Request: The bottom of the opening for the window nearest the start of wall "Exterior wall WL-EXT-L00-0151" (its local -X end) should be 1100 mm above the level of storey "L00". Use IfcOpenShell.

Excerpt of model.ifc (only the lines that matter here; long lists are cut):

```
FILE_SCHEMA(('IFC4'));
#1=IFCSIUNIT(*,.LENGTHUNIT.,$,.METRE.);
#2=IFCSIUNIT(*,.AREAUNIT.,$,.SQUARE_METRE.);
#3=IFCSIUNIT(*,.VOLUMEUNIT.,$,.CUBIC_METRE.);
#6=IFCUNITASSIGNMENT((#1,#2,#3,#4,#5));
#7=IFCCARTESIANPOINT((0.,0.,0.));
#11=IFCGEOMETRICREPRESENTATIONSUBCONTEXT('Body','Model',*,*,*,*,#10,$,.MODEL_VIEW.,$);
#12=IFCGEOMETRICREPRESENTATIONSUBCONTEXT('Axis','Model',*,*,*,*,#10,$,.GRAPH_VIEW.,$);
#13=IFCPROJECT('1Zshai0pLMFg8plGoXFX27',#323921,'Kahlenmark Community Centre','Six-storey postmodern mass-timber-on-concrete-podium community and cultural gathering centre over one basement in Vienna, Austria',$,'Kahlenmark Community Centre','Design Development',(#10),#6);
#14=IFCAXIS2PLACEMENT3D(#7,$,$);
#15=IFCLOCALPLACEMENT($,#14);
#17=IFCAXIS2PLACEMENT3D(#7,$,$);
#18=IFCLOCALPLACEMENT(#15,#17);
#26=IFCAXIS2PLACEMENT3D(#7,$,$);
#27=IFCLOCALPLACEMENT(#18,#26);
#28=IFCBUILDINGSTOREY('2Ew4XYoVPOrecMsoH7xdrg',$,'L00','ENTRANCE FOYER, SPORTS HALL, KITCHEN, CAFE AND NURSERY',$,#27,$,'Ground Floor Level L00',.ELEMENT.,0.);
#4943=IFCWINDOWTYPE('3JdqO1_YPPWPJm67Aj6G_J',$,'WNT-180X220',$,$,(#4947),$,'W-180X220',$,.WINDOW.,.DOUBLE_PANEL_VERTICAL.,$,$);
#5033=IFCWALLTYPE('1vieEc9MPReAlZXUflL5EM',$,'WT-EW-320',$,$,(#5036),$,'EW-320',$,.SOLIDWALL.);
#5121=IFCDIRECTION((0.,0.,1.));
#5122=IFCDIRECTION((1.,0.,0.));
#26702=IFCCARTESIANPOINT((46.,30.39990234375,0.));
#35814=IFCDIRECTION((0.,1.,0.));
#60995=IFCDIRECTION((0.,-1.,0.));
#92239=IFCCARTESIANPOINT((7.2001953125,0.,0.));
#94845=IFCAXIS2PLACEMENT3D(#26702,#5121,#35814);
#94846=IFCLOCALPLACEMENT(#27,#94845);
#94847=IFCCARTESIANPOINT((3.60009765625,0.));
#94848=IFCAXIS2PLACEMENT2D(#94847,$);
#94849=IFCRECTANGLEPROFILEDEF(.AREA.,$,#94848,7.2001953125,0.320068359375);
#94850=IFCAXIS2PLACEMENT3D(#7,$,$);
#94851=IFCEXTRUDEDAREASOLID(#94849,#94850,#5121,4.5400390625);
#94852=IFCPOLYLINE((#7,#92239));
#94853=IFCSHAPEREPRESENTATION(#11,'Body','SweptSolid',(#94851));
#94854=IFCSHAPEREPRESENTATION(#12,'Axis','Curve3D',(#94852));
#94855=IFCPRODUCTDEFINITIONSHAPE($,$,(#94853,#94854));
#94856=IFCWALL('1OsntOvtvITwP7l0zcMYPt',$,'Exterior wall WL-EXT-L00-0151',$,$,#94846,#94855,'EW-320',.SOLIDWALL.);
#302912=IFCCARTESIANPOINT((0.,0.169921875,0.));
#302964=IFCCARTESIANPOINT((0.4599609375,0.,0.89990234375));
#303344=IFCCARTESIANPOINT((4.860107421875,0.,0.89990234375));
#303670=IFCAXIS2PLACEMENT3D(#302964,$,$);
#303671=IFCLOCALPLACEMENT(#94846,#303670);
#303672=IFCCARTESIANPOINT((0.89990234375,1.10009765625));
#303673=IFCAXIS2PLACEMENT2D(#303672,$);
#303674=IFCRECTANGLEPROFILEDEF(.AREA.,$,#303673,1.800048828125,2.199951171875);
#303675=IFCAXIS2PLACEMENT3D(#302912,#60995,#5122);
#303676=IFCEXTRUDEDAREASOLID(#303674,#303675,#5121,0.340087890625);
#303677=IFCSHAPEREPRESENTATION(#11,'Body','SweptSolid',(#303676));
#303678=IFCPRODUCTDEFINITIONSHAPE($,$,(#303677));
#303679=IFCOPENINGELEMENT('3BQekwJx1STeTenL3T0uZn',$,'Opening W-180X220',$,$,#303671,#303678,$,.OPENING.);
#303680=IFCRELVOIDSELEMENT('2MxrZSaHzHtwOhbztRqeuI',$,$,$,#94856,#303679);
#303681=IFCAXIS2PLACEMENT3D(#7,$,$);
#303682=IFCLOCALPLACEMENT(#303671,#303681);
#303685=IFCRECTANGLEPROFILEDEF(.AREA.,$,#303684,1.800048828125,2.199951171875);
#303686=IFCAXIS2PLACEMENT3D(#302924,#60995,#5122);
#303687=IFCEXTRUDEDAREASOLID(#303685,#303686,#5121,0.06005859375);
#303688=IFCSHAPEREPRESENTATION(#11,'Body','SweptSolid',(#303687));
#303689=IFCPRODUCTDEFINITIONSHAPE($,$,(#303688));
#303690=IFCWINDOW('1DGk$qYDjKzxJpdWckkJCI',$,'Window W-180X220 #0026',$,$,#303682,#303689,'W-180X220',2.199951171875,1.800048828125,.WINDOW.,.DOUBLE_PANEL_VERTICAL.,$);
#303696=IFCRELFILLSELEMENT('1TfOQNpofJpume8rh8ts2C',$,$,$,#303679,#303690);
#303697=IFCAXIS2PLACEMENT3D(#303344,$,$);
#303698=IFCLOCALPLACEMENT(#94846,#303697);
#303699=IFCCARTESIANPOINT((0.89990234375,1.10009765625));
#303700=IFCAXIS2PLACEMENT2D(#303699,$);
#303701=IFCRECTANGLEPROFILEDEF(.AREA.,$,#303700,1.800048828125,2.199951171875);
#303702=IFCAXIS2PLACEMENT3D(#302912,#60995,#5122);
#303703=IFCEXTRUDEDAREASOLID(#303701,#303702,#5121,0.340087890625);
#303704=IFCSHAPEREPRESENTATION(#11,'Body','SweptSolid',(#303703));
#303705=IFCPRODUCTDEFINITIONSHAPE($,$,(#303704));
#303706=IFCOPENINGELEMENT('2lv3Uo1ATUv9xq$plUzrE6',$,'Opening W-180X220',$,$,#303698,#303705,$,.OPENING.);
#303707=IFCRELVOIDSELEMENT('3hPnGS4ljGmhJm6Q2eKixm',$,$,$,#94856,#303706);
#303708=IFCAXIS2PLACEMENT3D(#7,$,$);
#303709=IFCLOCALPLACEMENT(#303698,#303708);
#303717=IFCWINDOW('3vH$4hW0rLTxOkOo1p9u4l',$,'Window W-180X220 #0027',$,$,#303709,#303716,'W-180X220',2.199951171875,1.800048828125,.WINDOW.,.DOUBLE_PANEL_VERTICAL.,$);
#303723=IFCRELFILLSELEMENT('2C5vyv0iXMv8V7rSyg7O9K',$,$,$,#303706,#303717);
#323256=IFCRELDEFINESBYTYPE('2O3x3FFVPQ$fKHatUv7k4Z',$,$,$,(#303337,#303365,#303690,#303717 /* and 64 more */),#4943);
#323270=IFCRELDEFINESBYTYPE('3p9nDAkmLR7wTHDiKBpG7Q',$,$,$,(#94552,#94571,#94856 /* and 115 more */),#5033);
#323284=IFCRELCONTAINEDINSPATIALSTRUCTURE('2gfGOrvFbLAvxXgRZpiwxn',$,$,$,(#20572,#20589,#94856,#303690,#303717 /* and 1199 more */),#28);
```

```python
import numpy as np
import ifcopenshell
import ifcopenshell.api.geometry
import ifcopenshell.geom
import ifcopenshell.util.element
import ifcopenshell.util.placement
import ifcopenshell.util.shape
import ifcopenshell.util.unit

model = ifcopenshell.open("model.ifc")
unit_scale = ifcopenshell.util.unit.calculate_unit_scale(model)

window = model.by_guid("1DGk$qYDjKzxJpdWckkJCI")
opening = window.FillsVoids[0].RelatingOpeningElement
storey = ifcopenshell.util.element.get_container(window, ifc_class="IfcBuildingStorey")
level = ifcopenshell.util.placement.get_local_placement(storey.ObjectPlacement)[2, 3]

# The opening's origin need not be at the sill, so measure its lowest point.
shape = ifcopenshell.geom.create_shape(ifcopenshell.geom.settings(), opening)
bottom = ifcopenshell.util.shape.get_shape_bottom_elevation(shape, shape.geometry) / unit_scale
dz = level + 1.1 / unit_scale - bottom

shift = np.array([0.0, 0.0, dz])
# The window is placed relative to its opening, so it follows when the opening moves.
matrix = ifcopenshell.util.placement.get_local_placement(opening.ObjectPlacement)
matrix[:3, 3] += shift
ifcopenshell.api.geometry.edit_object_placement(
    model, product=opening, matrix=matrix, is_si=False, should_transform_children=True
)

print(f"moved by {dz * unit_scale:+.3f} m")

model.write("model_v2.ifc")
```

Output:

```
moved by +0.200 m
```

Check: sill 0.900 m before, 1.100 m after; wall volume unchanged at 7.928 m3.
